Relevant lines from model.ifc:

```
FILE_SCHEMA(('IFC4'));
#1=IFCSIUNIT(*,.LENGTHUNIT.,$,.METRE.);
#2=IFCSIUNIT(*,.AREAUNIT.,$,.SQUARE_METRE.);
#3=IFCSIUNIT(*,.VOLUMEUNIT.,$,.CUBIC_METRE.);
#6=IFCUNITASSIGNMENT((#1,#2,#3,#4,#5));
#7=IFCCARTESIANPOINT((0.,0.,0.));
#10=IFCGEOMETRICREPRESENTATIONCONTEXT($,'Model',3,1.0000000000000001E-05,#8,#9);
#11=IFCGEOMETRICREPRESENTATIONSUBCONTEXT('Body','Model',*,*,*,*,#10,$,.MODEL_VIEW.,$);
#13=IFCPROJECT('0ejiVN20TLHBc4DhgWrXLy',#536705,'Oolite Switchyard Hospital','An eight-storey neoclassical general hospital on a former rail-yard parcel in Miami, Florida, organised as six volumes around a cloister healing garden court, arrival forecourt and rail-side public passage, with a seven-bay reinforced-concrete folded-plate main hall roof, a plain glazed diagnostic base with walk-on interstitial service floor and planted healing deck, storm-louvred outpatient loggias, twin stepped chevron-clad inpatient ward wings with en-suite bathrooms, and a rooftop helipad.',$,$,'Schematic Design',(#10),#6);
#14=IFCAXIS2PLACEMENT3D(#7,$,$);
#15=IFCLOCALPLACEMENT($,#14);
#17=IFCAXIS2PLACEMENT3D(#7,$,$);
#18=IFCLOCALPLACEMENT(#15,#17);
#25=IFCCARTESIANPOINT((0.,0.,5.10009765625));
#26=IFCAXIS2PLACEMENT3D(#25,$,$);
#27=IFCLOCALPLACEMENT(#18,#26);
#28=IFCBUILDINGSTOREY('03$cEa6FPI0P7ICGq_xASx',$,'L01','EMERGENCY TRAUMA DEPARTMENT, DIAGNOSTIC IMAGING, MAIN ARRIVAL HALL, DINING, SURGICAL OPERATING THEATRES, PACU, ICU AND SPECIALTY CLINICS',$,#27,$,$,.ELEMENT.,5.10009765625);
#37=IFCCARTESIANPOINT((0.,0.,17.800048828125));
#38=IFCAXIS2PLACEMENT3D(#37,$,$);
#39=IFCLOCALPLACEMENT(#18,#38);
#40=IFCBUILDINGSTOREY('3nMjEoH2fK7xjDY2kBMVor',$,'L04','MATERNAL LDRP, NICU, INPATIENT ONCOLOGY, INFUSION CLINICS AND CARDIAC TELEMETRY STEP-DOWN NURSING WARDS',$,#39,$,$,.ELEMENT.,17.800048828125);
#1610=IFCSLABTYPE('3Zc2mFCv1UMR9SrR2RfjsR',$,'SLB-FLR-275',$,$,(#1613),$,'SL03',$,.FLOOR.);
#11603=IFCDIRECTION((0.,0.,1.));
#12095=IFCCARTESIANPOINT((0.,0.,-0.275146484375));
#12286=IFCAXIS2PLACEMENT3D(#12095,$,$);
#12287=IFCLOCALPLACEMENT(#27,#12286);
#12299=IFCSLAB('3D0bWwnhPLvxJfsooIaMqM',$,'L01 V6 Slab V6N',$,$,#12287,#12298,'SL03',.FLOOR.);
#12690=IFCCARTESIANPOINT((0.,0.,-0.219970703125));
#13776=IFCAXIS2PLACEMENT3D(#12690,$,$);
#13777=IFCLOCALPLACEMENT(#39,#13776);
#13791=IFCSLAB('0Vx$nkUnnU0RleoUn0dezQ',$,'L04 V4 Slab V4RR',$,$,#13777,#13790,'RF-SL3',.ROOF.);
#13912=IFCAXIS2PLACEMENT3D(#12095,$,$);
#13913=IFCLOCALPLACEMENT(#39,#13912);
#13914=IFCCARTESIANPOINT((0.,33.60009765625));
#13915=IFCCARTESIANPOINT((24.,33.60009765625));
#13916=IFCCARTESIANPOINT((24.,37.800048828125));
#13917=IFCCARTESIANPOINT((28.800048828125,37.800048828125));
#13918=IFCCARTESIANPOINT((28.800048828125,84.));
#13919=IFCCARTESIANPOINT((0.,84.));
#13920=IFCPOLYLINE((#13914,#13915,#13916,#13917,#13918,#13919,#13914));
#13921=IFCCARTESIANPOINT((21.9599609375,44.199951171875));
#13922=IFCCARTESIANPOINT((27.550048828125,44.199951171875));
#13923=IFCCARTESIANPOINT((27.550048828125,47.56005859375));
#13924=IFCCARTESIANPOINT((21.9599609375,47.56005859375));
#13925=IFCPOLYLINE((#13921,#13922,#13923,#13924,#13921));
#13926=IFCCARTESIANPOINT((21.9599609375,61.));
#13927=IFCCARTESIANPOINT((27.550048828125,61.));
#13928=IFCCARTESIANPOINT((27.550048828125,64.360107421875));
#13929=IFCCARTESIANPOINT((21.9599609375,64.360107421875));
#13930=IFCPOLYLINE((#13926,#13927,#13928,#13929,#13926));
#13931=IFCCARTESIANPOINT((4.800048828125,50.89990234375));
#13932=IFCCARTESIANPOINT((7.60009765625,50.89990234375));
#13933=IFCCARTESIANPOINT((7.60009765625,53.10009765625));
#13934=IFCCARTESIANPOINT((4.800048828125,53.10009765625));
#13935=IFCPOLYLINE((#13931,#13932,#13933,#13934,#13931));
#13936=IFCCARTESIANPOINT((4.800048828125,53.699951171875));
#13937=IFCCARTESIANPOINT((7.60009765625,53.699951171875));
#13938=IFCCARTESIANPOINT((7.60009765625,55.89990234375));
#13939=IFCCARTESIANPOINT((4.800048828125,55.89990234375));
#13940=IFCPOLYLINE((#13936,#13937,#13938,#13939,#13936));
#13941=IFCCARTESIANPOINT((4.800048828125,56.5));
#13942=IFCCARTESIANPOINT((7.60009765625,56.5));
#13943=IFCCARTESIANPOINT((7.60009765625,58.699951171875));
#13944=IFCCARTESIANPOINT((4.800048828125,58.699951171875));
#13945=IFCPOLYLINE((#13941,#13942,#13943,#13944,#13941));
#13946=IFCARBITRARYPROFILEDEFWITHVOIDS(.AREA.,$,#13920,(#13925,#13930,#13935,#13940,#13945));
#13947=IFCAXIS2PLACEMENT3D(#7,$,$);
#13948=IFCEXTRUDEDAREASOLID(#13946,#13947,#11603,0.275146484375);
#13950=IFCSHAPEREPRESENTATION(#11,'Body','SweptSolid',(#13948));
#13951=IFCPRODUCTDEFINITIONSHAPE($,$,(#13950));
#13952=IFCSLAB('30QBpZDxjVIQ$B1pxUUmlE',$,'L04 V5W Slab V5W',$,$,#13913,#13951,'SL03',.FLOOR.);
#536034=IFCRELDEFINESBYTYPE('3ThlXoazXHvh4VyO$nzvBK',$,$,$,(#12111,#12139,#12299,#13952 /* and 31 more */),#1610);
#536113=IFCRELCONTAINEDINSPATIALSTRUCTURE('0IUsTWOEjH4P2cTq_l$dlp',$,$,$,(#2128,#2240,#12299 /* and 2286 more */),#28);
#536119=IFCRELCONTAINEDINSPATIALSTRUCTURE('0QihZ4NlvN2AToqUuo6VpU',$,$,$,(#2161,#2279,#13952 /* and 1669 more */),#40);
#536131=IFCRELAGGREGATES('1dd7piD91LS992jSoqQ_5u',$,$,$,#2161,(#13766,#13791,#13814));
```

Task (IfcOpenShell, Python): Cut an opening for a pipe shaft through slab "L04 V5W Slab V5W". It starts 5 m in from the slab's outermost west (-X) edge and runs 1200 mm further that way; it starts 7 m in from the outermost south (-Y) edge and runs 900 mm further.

```python
import numpy as np
import ifcopenshell
import ifcopenshell.api.feature
import ifcopenshell.api.geometry
import ifcopenshell.api.root
import ifcopenshell.geom
import ifcopenshell.util.placement
import ifcopenshell.util.representation
import ifcopenshell.util.shape
import ifcopenshell.util.unit

model = ifcopenshell.open("model.ifc")
unit_scale = ifcopenshell.util.unit.calculate_unit_scale(model)
settings = ifcopenshell.geom.settings()


def volume(element):
    """Net volume in cubic metres, openings subtracted."""
    shape = ifcopenshell.geom.create_shape(settings, element)
    return ifcopenshell.util.shape.get_volume(shape.geometry)


slab = model.by_guid("30QBpZDxjVIQ$B1pxUUmlE")
before = volume(slab)

# Extent in the slab's own axes, in metres. The edges named are its -X and -Y sides.
slab_shape = ifcopenshell.geom.create_shape(settings, slab)
vertices = ifcopenshell.util.shape.get_vertices(slab_shape.geometry)
x_min, y_min, bottom = vertices.min(axis=0)
top = vertices[:, 2].max()

opening = ifcopenshell.api.root.create_entity(model, ifc_class="IfcOpeningElement", name="Pipe shaft opening", predefined_type="OPENING")
context = ifcopenshell.util.representation.get_context(model, "Model", "Body", "MODEL_VIEW")
width, depth = 1.2, 0.9
outline = [(0.0, 0.0), (width, 0.0), (width, depth), (0.0, depth), (0.0, 0.0)]
# Overshoot both faces by 50 mm so the cut is clean.
shape = ifcopenshell.api.geometry.add_slab_representation(
    model, context=context, depth=top - bottom + 0.1, polyline=outline
)
ifcopenshell.api.geometry.assign_representation(model, product=opening, representation=shape)

matrix = ifcopenshell.util.placement.get_local_placement(slab.ObjectPlacement)
matrix[:, 3] = matrix @ np.append(np.array([x_min + 5, y_min + 7, bottom - 0.05]) / unit_scale, 1.0)
ifcopenshell.api.geometry.edit_object_placement(model, product=opening, matrix=matrix, is_si=False)
ifcopenshell.api.feature.add_feature(model, feature=opening, element=slab)

after = volume(slab)

print(f"slab volume {before:.3f} -> {after:.3f} m3")

model.write("model_rev.ifc")
```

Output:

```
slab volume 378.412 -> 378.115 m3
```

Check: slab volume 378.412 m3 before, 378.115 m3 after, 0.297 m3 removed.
